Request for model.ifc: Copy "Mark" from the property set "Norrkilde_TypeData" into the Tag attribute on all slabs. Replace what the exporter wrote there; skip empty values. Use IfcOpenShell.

First a look at what the model holds.

```python
import ifcopenshell
import ifcopenshell.util.element

model = ifcopenshell.open("model.ifc")
print(model.schema)
slabs = model.by_type("IfcSlab")
print(len(slabs), "slabs")
for e in slabs[:8]:
    source = ifcopenshell.util.element.get_pset(e, "Norrkilde_TypeData", "Mark")
    target = e.Tag
    print(e.id(), repr(source), repr(target), sep=" | ")
```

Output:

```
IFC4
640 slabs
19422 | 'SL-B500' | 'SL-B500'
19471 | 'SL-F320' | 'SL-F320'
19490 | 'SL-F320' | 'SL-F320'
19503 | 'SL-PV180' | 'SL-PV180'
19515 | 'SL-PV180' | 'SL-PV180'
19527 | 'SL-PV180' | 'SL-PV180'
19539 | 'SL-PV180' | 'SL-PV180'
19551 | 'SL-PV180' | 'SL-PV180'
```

```python
import ifcopenshell
import ifcopenshell.util.element

model = ifcopenshell.open("model.ifc")

count = 0
for e in model.by_type("IfcSlab"):
    value = ifcopenshell.util.element.get_pset(e, "Norrkilde_TypeData", "Mark")
    current = e.Tag
    if not value or not value.strip() or current == value:
        continue
    e.Tag = value
    count += 1

print(count, "slabs updated")

model.write("model-out.ifc")
```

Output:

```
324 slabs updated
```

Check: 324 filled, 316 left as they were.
